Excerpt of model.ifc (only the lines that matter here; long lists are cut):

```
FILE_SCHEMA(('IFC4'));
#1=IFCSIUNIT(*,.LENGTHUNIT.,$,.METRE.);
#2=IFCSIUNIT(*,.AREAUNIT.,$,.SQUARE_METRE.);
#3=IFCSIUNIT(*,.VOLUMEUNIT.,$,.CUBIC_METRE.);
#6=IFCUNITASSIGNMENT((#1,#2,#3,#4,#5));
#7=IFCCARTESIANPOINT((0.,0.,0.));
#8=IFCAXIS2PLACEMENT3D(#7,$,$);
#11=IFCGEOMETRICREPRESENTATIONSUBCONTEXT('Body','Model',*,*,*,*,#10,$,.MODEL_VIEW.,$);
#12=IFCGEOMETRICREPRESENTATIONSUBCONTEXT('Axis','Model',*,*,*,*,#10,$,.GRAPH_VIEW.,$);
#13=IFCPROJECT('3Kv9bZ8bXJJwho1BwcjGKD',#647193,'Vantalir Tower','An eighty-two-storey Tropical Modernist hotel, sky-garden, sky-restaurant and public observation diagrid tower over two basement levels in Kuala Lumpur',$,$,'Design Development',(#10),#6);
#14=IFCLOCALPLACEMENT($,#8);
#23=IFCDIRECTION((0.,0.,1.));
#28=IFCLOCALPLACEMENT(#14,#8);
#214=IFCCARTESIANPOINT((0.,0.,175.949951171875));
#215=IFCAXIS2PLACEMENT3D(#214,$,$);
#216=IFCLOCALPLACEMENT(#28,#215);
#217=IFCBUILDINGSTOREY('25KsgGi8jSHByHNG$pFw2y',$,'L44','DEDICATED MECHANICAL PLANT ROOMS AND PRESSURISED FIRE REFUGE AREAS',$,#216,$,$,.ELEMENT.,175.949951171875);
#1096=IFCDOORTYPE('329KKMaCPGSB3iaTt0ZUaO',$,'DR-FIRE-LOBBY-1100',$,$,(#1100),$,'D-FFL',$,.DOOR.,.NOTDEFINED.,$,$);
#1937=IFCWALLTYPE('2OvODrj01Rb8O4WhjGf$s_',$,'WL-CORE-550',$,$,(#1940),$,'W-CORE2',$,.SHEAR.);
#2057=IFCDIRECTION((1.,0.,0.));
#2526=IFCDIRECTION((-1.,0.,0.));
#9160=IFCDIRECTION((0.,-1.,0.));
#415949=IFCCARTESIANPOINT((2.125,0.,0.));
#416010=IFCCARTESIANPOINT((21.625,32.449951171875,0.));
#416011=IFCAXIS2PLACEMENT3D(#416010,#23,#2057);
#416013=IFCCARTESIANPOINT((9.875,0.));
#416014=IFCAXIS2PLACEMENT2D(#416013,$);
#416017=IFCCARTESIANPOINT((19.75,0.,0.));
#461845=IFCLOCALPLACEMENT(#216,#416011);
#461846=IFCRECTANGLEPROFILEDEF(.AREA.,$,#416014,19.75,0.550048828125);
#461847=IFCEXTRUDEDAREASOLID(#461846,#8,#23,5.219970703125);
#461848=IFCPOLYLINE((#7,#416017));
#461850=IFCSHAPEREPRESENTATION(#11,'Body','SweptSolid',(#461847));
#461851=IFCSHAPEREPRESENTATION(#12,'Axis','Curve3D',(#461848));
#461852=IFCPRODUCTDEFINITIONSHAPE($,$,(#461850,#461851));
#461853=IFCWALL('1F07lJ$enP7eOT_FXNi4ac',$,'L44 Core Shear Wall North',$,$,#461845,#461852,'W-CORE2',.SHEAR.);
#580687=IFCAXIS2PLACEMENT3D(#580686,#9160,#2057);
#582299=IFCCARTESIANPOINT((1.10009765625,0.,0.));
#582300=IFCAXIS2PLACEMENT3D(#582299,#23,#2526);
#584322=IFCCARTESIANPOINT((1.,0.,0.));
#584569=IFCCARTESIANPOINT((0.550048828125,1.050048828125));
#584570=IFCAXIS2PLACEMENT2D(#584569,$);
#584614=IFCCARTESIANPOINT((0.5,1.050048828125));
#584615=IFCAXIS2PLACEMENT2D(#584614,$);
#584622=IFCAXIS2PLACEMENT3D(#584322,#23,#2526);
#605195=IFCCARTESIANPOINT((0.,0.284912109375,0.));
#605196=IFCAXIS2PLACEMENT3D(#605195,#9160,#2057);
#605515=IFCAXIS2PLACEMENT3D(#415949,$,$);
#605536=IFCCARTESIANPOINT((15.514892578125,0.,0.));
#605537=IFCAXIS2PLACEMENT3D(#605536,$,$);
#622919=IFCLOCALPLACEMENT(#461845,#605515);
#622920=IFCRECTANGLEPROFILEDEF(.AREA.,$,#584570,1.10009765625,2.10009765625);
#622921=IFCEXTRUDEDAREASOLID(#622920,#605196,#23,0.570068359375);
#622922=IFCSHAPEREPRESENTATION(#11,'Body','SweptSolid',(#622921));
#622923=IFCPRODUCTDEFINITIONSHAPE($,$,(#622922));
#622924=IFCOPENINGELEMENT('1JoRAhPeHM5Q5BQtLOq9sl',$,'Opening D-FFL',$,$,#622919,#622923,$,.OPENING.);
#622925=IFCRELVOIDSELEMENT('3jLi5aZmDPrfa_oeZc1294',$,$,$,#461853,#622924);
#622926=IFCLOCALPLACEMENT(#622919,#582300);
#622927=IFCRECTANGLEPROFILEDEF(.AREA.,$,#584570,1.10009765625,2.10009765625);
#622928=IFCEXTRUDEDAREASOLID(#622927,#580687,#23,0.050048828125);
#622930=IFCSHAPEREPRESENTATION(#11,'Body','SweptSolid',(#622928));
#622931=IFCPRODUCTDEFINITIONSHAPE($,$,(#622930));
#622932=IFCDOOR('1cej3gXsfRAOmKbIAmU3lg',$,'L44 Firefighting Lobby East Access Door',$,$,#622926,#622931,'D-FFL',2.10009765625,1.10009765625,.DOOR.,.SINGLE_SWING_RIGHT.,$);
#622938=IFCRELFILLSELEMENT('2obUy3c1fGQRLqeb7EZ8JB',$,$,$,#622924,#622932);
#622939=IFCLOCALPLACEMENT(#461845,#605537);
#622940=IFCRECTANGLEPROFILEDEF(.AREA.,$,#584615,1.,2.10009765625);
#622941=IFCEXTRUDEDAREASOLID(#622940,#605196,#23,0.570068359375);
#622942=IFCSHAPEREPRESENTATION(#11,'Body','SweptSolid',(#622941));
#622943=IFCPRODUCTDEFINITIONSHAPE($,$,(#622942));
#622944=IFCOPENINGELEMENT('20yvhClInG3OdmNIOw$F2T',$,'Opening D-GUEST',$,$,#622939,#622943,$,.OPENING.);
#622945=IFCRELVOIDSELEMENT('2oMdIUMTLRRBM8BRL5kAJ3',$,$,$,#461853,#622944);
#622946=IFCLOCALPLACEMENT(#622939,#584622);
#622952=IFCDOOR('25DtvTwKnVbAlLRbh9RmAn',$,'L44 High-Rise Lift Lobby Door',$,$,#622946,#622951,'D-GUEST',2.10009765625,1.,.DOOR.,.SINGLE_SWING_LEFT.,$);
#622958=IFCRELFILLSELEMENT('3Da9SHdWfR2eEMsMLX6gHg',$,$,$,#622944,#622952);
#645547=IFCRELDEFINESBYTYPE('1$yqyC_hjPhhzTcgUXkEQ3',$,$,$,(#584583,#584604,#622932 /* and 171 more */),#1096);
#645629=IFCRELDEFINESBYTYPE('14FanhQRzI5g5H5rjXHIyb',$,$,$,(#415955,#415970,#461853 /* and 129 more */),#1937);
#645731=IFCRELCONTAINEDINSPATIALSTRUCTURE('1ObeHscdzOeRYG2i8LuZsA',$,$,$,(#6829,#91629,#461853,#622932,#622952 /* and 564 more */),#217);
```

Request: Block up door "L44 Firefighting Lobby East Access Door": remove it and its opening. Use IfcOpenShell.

```python
import ifcopenshell
import ifcopenshell.api.feature
import ifcopenshell.api.root
import ifcopenshell.geom
import ifcopenshell.util.shape

model = ifcopenshell.open("model.ifc")
settings = ifcopenshell.geom.settings()


def volume(element):
    """Net volume in cubic metres, openings subtracted."""
    shape = ifcopenshell.geom.create_shape(settings, element)
    return ifcopenshell.util.shape.get_volume(shape.geometry)


door = model.by_guid("1cej3gXsfRAOmKbIAmU3lg")
opening = door.FillsVoids[0].RelatingOpeningElement
wall = opening.VoidsElements[0].RelatingBuildingElement
before = volume(wall)

ifcopenshell.api.root.remove_product(model, product=door)
ifcopenshell.api.feature.remove_feature(model, feature=opening)

after = volume(wall)

print(f"wall volume {before:.3f} -> {after:.3f} m3")

model.write("model-out.ifc")
```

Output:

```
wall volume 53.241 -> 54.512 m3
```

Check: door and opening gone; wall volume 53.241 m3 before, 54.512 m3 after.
